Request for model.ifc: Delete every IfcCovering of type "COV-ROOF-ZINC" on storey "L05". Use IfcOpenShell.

First a look at what the model holds.

```python
import ifcopenshell
import ifcopenshell.util.element

model = ifcopenshell.open("model.ifc")
print(model.schema)
storey = next(s for s in model.by_type("IfcBuildingStorey") if s.Name == "L05")
coverings = [e for e in ifcopenshell.util.element.get_decomposition(storey) if e.is_a("IfcCovering")]
seen = {}
for e in coverings:
    element_type = ifcopenshell.util.element.get_type(e)
    name = element_type.Name if element_type not in (None, e) else None
    seen[name] = seen.get(name, 0) + 1
for name, count in sorted(seen.items(), key=str):
    print(count, "x", name)
```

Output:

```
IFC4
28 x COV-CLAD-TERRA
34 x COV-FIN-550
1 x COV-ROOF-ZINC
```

```python
import ifcopenshell
import ifcopenshell.api.root
import ifcopenshell.util.element

model = ifcopenshell.open("model.ifc")

storey = next(s for s in model.by_type("IfcBuildingStorey") if s.Name == "L05")
coverings = [e for e in ifcopenshell.util.element.get_decomposition(storey) if e.is_a("IfcCovering")]
targets = [e for e in coverings if (t := ifcopenshell.util.element.get_type(e)) not in (None, e) and t.Name == "COV-ROOF-ZINC"]

for e in targets:
    ifcopenshell.api.root.remove_product(model, product=e)
print(len(targets), "removed")

model.write("model_updated.ifc")
```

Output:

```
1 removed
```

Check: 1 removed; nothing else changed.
